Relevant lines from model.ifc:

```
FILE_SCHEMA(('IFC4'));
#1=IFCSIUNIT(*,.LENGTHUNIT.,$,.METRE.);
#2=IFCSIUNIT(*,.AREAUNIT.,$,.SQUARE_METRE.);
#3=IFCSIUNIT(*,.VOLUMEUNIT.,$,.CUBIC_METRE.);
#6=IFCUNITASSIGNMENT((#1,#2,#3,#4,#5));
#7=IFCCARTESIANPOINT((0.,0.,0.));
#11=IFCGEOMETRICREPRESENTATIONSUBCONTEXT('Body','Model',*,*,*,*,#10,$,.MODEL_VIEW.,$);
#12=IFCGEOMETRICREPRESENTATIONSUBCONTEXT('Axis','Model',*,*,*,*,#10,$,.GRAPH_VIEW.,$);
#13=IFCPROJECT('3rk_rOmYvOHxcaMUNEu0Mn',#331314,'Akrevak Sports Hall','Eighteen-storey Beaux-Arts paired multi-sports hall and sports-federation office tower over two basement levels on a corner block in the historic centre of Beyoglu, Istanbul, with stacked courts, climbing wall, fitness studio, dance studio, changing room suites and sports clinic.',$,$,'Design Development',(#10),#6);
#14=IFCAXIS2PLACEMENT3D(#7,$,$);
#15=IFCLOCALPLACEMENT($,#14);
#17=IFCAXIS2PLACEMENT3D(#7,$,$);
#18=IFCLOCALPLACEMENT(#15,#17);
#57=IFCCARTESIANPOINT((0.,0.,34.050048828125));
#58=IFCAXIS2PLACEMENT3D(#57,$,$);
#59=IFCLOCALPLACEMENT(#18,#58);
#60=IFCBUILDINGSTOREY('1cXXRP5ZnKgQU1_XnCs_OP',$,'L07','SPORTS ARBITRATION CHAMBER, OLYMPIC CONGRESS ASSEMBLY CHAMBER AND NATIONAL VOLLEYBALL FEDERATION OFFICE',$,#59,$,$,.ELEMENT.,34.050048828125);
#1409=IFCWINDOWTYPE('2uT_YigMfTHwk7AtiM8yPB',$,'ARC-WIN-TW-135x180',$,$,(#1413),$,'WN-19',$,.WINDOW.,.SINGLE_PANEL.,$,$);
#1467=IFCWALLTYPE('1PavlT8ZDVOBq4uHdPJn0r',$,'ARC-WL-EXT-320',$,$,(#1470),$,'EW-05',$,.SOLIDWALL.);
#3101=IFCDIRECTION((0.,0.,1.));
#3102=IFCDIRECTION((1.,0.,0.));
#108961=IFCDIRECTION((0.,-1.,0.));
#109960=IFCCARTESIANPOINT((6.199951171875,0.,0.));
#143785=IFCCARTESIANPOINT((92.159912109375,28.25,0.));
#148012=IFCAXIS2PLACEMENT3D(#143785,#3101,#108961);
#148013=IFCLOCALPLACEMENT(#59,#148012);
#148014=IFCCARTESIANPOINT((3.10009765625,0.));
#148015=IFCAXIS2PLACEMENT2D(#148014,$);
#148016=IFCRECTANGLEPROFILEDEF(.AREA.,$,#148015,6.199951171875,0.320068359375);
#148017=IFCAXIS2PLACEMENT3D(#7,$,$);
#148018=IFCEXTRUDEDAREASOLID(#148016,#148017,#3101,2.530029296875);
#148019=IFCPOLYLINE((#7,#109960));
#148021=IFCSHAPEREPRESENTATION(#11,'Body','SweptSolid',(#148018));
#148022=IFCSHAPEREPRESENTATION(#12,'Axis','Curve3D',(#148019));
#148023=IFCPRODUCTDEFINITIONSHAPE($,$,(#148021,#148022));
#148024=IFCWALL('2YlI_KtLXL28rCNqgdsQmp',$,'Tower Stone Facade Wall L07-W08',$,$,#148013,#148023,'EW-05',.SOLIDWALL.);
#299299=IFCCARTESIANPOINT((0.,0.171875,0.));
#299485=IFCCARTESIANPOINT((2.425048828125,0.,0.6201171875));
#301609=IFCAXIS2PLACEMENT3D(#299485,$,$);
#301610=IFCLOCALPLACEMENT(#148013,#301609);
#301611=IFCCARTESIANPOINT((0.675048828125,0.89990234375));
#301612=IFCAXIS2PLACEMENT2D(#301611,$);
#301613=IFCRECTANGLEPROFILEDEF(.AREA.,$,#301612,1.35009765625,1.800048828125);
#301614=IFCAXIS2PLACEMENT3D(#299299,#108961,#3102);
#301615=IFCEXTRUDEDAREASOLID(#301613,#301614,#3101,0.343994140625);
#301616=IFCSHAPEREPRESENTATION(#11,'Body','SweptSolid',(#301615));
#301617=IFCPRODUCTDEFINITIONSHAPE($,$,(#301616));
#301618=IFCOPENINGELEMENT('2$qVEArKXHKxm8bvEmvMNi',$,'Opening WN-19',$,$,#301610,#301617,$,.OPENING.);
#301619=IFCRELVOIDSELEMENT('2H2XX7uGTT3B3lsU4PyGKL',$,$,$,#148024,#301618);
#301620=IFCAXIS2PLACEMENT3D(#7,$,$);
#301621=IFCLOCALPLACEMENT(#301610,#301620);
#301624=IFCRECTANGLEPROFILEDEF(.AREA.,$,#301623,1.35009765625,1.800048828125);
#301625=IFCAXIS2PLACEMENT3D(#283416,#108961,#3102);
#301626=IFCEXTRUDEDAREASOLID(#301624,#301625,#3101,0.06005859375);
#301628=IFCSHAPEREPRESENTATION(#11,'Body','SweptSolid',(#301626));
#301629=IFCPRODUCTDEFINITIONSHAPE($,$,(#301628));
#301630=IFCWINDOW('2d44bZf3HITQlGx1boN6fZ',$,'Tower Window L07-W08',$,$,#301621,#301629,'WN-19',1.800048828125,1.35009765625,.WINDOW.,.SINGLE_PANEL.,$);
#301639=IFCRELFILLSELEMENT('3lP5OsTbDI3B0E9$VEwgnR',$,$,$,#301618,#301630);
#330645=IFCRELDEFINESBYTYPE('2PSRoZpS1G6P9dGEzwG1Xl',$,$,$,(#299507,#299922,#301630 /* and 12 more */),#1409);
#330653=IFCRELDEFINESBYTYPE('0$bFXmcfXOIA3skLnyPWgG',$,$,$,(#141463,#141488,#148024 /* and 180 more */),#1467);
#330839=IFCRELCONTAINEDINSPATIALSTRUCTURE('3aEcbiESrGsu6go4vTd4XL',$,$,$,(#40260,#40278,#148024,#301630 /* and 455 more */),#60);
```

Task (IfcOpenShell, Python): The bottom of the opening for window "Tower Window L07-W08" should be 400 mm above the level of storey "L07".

```python
import numpy as np
import ifcopenshell
import ifcopenshell.api.geometry
import ifcopenshell.geom
import ifcopenshell.util.element
import ifcopenshell.util.placement
import ifcopenshell.util.shape
import ifcopenshell.util.unit

model = ifcopenshell.open("model.ifc")
unit_scale = ifcopenshell.util.unit.calculate_unit_scale(model)

window = model.by_guid("2d44bZf3HITQlGx1boN6fZ")
opening = window.FillsVoids[0].RelatingOpeningElement
storey = ifcopenshell.util.element.get_container(window, ifc_class="IfcBuildingStorey")
level = ifcopenshell.util.placement.get_local_placement(storey.ObjectPlacement)[2, 3]

# The opening's origin need not be at the sill, so measure its lowest point.
shape = ifcopenshell.geom.create_shape(ifcopenshell.geom.settings(), opening)
bottom = ifcopenshell.util.shape.get_shape_bottom_elevation(shape, shape.geometry) / unit_scale
dz = level + 0.4 / unit_scale - bottom

shift = np.array([0.0, 0.0, dz])
# The window is placed relative to its opening, so it follows when the opening moves.
matrix = ifcopenshell.util.placement.get_local_placement(opening.ObjectPlacement)
matrix[:3, 3] += shift
ifcopenshell.api.geometry.edit_object_placement(
    model, product=opening, matrix=matrix, is_si=False, should_transform_children=True
)

print(f"moved by {dz * unit_scale:+.3f} m")

model.write("model_edited.ifc")
```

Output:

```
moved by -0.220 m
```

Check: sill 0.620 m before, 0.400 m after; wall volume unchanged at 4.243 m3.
